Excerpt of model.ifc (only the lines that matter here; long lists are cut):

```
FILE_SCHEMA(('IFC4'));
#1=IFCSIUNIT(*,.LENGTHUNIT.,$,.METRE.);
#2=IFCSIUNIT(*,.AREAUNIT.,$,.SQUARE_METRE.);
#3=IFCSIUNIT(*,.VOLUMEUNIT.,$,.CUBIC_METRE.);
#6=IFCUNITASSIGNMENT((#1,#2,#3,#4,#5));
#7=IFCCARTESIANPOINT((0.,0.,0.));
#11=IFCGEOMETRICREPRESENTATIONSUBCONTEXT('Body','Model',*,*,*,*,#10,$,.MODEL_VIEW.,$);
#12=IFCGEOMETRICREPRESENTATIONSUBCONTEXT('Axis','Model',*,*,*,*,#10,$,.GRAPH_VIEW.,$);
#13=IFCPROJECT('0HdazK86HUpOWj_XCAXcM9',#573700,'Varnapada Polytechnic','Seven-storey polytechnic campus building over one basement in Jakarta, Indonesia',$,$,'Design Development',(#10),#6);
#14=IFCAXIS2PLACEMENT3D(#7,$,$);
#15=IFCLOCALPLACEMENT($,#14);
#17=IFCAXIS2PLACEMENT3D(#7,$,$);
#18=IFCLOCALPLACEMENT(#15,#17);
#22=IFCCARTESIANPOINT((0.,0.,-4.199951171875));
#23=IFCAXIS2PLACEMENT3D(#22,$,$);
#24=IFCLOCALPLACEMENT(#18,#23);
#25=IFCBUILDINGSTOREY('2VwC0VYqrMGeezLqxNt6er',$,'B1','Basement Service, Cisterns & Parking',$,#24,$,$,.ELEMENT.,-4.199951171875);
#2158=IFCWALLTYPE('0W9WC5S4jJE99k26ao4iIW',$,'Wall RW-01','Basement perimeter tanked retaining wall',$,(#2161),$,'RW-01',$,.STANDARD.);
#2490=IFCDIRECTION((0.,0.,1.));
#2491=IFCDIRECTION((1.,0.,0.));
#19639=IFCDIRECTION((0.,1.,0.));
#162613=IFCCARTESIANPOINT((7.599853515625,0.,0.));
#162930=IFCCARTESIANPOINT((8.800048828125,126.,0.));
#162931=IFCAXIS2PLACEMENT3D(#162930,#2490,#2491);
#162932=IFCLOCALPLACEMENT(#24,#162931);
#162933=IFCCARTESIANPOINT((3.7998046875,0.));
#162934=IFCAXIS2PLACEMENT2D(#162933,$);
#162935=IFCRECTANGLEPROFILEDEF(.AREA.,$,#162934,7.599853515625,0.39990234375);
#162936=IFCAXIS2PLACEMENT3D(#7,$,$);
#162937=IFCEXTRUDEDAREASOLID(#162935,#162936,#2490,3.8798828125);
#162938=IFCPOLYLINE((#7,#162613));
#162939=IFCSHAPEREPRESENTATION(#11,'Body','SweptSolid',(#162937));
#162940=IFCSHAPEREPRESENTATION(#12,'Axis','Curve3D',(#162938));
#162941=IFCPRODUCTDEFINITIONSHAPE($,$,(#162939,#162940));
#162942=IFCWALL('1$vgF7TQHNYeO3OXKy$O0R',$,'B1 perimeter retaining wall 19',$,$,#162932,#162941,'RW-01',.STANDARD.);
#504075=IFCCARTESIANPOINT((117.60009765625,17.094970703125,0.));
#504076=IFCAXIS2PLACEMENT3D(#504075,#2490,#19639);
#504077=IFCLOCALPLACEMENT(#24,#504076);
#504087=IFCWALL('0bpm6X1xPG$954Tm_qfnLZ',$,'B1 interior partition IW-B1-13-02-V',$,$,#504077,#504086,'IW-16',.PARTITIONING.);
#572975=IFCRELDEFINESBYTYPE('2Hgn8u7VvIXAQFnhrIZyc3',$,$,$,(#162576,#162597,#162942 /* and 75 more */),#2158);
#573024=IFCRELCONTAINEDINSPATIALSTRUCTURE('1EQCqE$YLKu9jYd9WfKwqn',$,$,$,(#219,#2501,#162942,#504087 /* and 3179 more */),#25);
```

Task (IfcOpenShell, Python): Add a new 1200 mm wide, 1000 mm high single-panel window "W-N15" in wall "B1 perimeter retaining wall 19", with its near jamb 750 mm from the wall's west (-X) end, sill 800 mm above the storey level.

```python
import numpy as np
import ifcopenshell
import ifcopenshell.api.feature
import ifcopenshell.api.geometry
import ifcopenshell.api.root
import ifcopenshell.api.spatial
import ifcopenshell.geom
import ifcopenshell.util.element
import ifcopenshell.util.placement
import ifcopenshell.util.representation
import ifcopenshell.util.shape
import ifcopenshell.util.unit

model = ifcopenshell.open("model.ifc")
unit_scale = ifcopenshell.util.unit.calculate_unit_scale(model)
settings = ifcopenshell.geom.settings()


def volume(element):
    """Net volume in cubic metres, openings subtracted."""
    shape = ifcopenshell.geom.create_shape(settings, element)
    return ifcopenshell.util.shape.get_volume(shape.geometry)


wall = model.by_guid("1$vgF7TQHNYeO3OXKy$O0R")
storey = ifcopenshell.util.element.get_container(wall, ifc_class="IfcBuildingStorey")
context = ifcopenshell.util.representation.get_context(model, "Model", "Body", "MODEL_VIEW")
before = volume(wall)

width, height, from_end, sill = 1.2, 1, 0.75, 0.8  # metres

# The wall runs along its own X axis, and the end named is its -X end.
wall_shape = ifcopenshell.geom.create_shape(settings, wall)
x, y, z = ifcopenshell.util.shape.get_vertices(wall_shape.geometry).T
start = x.min() + from_end
face, thickness = float(y.min()), float(y.max() - y.min())
wall_matrix = ifcopenshell.util.placement.get_local_placement(wall.ObjectPlacement)
level = ifcopenshell.util.placement.get_local_placement(storey.ObjectPlacement)[2, 3]


def in_wall(x, y):
    """Placement at x, y metres in the wall's axes, at sill height."""
    matrix = wall_matrix.copy()
    matrix[:, 3] = wall_matrix @ np.array([x / unit_scale, y / unit_scale, 0.0, 1.0])
    matrix[2, 3] = level + sill / unit_scale
    return matrix


# Opening: a box that overshoots both wall faces by 50 mm.
opening = ifcopenshell.api.root.create_entity(model, ifc_class="IfcOpeningElement", predefined_type="OPENING")
box = ifcopenshell.api.geometry.add_wall_representation(
    model, context=context, length=width, height=height, thickness=thickness + 0.1
)
ifcopenshell.api.geometry.assign_representation(model, product=opening, representation=box)
ifcopenshell.api.geometry.edit_object_placement(model, product=opening, matrix=in_wall(start, face - 0.05), is_si=False)
ifcopenshell.api.feature.add_feature(model, feature=opening, element=wall)

window = ifcopenshell.api.root.create_entity(model, ifc_class="IfcWindow", name="W-N15", predefined_type="WINDOW")
window.OverallWidth, window.OverallHeight = width / unit_scale, height / unit_scale
window.PartitioningType = "SINGLE_PANEL"
body = ifcopenshell.api.geometry.add_window_representation(
    model,
    context=context,
    overall_width=window.OverallWidth,
    overall_height=window.OverallHeight,
    partition_type="SINGLE_PANEL",
)
ifcopenshell.api.geometry.assign_representation(model, product=window, representation=body)
ifcopenshell.api.spatial.assign_container(model, products=[window], relating_structure=storey)
ifcopenshell.api.feature.add_filling(model, opening=opening, element=window)

# Centre the window in the wall's thickness.
ifcopenshell.api.geometry.edit_object_placement(model, product=window, matrix=in_wall(start, face), is_si=False)
window_shape = ifcopenshell.geom.create_shape(settings, window)
depth = ifcopenshell.util.shape.get_vertices(window_shape.geometry)[:, 1]
offset = face + thickness / 2 - (depth.min() + depth.max()) / 2
ifcopenshell.api.geometry.edit_object_placement(model, product=window, matrix=in_wall(start, offset), is_si=False)

after = volume(wall)

print(f"wall volume {before:.3f} -> {after:.3f} m3")

model.write("model_v2.ifc")
```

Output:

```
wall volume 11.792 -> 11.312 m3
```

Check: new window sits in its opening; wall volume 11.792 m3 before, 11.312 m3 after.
